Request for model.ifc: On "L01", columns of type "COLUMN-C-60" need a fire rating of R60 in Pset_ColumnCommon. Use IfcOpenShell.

First a look at what the model holds.

```python
import ifcopenshell
import ifcopenshell.util.element

model = ifcopenshell.open("model.ifc")
print(model.schema)
storey = next(s for s in model.by_type("IfcBuildingStorey") if s.Name == "L01")
columns = [e for e in ifcopenshell.util.element.get_decomposition(storey) if e.is_a("IfcColumn")]
seen = {}
for e in columns:
    element_type = ifcopenshell.util.element.get_type(e)
    key = (element_type.Name if element_type != e and element_type else None, ifcopenshell.util.element.get_pset(e, "Pset_ColumnCommon", "FireRating"))
    seen[key] = seen.get(key, 0) + 1
for (name, value), count in sorted(seen.items(), key=str):
    print(count, "x", name, "|", value)
```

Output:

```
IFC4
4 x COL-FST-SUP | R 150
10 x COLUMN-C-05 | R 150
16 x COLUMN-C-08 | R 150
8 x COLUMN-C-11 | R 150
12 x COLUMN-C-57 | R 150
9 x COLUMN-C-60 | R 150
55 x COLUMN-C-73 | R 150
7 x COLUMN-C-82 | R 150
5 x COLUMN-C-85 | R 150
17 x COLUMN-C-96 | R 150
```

```python
import ifcopenshell
import ifcopenshell.api.pset
import ifcopenshell.util.element

model = ifcopenshell.open("model.ifc")

storey = next(s for s in model.by_type("IfcBuildingStorey") if s.Name == "L01")
columns = [e for e in ifcopenshell.util.element.get_decomposition(storey) if e.is_a("IfcColumn")]

count = 0
for e in columns:
    element_type = ifcopenshell.util.element.get_type(e)
    if element_type in (None, e) or element_type.Name != "COLUMN-C-60":
        continue
    # add_pset returns the element's existing set when there is one.
    pset = ifcopenshell.api.pset.add_pset(model, product=e, name="Pset_ColumnCommon")
    ifcopenshell.api.pset.edit_pset(model, pset=pset, properties={"FireRating": "R60"})
    count += 1

print(count, "columns updated")

model.write("model_edited.ifc")
```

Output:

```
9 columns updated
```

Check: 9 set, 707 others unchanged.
